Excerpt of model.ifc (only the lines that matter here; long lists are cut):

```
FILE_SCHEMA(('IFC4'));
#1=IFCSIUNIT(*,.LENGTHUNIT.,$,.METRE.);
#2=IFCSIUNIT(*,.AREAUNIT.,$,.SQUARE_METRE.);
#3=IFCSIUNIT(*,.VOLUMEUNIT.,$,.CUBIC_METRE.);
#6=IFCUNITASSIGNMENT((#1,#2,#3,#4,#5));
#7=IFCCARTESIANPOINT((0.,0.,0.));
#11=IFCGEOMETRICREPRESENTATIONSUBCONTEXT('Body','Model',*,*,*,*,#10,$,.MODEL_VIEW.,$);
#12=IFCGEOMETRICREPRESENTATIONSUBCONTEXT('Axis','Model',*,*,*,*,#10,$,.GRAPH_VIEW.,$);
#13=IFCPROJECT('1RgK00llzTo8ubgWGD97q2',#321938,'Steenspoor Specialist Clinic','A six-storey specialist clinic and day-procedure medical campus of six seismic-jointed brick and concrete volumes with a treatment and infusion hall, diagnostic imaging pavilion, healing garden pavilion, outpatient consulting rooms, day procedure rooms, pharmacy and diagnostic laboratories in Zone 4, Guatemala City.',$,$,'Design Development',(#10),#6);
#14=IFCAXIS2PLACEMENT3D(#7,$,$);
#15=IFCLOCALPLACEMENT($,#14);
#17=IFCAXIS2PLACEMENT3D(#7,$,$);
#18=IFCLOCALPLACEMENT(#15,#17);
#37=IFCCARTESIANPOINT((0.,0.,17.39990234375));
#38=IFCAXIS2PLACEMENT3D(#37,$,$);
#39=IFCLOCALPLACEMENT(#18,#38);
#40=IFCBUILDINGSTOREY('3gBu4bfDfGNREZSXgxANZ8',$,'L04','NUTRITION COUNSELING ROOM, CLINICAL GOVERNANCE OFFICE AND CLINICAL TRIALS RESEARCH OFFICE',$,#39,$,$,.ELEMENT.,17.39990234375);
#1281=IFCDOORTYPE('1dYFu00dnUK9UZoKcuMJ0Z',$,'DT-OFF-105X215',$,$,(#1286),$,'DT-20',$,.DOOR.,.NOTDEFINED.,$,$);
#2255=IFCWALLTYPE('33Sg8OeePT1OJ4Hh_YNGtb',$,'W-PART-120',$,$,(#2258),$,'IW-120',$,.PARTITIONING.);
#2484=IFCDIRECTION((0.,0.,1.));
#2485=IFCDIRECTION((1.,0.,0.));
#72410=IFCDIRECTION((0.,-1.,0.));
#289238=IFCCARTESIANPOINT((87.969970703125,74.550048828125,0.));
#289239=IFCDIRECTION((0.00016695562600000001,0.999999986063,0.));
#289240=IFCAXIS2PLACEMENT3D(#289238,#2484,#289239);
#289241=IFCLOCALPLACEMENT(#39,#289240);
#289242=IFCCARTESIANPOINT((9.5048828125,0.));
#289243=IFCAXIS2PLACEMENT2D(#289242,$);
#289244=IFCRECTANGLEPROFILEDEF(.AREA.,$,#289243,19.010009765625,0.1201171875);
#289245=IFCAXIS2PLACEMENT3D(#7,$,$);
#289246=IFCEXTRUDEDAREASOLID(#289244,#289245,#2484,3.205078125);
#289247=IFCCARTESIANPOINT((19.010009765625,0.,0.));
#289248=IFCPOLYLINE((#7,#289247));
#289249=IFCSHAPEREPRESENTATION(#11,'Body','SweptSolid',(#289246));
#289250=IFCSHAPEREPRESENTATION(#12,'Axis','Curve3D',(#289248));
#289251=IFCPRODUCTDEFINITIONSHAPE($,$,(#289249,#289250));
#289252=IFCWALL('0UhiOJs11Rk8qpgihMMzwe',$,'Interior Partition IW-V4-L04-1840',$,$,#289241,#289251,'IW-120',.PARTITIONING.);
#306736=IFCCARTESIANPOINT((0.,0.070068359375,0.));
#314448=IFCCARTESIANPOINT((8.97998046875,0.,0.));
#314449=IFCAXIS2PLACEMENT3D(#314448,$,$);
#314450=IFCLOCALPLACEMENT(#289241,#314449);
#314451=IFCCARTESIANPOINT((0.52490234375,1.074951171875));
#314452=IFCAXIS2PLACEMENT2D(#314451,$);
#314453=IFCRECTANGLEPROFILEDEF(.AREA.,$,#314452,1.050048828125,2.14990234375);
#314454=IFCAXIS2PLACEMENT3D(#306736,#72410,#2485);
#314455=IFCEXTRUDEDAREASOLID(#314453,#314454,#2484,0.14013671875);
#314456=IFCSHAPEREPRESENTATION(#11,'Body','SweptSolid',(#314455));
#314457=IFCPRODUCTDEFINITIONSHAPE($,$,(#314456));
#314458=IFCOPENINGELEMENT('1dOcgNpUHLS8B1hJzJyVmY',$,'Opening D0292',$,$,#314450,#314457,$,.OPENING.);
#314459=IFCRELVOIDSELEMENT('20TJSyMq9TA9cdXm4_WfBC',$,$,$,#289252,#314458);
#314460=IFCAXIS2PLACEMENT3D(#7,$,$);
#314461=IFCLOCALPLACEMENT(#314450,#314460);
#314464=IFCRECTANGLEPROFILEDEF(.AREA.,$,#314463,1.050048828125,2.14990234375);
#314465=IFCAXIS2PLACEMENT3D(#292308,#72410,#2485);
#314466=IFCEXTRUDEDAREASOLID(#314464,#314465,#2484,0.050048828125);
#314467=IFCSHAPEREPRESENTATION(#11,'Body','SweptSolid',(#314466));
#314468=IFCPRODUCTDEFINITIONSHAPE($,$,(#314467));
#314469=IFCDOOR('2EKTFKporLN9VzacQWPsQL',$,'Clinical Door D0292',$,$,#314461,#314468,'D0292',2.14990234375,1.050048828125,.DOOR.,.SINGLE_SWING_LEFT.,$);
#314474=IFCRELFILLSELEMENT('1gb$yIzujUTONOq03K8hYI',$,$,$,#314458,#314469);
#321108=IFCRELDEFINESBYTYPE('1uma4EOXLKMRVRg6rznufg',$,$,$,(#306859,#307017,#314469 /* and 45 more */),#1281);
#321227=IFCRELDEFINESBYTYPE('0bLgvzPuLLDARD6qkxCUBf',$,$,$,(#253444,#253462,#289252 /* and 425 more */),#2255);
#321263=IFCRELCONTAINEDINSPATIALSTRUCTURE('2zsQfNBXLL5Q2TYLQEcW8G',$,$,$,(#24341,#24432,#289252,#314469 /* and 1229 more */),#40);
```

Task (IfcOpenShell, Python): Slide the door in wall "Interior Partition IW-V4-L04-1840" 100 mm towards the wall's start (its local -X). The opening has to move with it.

```python
import ifcopenshell
import ifcopenshell.api.geometry
import ifcopenshell.util.placement

model = ifcopenshell.open("model.ifc")

door = model.by_guid("2EKTFKporLN9VzacQWPsQL")
opening = door.FillsVoids[0].RelatingOpeningElement
wall = opening.VoidsElements[0].RelatingBuildingElement

wall_matrix = ifcopenshell.util.placement.get_local_placement(wall.ObjectPlacement)
shift = wall_matrix[:3, 0] * -0.1
before = ifcopenshell.util.placement.get_local_placement(door.ObjectPlacement)[:3, 3].copy()

# The door is placed relative to its opening, so it follows when the opening moves.
matrix = ifcopenshell.util.placement.get_local_placement(opening.ObjectPlacement)
matrix[:3, 3] += shift
ifcopenshell.api.geometry.edit_object_placement(
    model, product=opening, matrix=matrix, is_si=False, should_transform_children=True
)

after = ifcopenshell.util.placement.get_local_placement(door.ObjectPlacement)[:3, 3]
print("door moved by", (after - before).round(3) + 0.0)

model.write("model_updated.ifc")
```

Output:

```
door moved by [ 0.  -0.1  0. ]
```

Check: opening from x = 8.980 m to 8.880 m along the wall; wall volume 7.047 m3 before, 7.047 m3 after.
